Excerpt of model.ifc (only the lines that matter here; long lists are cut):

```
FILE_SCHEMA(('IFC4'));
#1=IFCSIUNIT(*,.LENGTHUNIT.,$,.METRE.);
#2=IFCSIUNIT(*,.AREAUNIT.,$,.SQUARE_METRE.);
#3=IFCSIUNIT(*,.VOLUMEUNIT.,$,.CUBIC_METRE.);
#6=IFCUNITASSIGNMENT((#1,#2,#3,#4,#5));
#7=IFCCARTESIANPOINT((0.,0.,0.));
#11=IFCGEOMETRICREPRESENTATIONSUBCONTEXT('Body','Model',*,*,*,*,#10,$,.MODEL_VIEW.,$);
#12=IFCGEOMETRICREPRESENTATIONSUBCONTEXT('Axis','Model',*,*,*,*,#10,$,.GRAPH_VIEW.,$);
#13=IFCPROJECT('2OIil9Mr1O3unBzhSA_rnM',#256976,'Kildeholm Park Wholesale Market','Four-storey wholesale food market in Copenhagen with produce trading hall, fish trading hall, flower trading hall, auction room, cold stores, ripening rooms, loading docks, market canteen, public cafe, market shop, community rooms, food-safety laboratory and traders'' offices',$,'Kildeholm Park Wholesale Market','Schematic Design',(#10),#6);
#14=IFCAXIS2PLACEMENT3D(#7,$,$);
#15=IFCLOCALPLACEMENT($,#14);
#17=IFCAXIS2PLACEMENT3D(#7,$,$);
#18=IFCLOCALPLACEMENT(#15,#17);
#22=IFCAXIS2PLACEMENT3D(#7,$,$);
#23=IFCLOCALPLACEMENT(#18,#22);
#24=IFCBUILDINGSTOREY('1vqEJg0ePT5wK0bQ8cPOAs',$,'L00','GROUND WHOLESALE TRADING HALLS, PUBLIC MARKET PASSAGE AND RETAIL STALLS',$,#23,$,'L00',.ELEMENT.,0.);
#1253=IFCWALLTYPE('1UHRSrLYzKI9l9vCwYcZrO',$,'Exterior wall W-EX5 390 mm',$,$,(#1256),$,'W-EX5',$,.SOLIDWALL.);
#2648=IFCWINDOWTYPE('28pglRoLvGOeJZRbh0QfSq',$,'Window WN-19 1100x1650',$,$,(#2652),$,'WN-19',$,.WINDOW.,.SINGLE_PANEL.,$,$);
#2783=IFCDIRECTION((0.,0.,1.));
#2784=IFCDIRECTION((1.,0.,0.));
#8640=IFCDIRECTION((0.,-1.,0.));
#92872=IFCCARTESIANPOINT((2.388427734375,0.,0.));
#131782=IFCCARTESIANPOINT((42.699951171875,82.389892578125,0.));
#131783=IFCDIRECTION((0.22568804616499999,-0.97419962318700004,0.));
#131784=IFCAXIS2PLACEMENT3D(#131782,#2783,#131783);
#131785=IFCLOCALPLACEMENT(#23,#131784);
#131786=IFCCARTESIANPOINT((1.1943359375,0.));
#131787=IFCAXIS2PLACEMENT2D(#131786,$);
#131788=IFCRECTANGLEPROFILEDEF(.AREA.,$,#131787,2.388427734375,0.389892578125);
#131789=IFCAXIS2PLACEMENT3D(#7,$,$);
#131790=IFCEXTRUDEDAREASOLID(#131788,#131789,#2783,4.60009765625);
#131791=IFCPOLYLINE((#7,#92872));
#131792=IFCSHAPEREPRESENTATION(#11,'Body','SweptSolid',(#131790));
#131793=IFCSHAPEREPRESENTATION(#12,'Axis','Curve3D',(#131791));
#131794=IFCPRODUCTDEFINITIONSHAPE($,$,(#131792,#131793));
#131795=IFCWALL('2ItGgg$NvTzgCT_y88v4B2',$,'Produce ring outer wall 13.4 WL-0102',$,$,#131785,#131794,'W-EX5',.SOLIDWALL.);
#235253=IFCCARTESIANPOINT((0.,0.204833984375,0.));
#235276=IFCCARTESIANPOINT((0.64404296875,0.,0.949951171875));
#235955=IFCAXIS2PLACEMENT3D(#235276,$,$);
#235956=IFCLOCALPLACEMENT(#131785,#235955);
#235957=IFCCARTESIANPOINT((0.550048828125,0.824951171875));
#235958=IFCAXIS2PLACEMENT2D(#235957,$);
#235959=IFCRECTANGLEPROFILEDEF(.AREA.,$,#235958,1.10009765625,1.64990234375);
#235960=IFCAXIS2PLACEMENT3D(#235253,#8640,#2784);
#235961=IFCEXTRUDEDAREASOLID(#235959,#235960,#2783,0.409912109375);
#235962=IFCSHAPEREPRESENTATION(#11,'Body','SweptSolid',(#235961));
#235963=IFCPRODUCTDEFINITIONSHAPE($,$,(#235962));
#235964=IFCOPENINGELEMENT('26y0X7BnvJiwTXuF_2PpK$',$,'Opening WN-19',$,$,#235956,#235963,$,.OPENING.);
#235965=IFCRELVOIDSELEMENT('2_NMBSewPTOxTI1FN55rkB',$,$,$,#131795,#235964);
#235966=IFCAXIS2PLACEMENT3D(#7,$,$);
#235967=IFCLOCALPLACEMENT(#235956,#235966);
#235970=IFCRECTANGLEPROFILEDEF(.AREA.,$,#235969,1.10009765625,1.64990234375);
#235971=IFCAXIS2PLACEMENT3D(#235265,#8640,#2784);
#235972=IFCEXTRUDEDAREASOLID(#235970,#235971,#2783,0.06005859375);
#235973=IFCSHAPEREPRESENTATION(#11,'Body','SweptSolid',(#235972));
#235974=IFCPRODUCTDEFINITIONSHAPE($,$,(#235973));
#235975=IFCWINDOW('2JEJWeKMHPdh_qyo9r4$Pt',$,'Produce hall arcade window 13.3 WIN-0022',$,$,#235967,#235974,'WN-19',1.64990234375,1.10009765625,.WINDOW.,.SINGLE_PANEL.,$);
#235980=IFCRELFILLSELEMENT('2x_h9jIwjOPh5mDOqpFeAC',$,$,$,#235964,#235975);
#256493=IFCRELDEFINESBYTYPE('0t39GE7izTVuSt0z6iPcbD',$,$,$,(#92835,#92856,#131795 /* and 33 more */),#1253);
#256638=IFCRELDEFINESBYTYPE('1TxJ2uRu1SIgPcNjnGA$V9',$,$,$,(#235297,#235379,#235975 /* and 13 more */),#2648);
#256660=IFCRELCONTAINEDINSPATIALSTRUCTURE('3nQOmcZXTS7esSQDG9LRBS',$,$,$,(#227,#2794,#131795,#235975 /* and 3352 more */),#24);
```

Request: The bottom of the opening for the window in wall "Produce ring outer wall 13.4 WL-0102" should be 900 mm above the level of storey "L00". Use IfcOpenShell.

```python
import numpy as np
import ifcopenshell
import ifcopenshell.api.geometry
import ifcopenshell.geom
import ifcopenshell.util.element
import ifcopenshell.util.placement
import ifcopenshell.util.shape
import ifcopenshell.util.unit

model = ifcopenshell.open("model.ifc")
unit_scale = ifcopenshell.util.unit.calculate_unit_scale(model)

window = model.by_guid("2JEJWeKMHPdh_qyo9r4$Pt")
opening = window.FillsVoids[0].RelatingOpeningElement
storey = ifcopenshell.util.element.get_container(window, ifc_class="IfcBuildingStorey")
level = ifcopenshell.util.placement.get_local_placement(storey.ObjectPlacement)[2, 3]

# The opening's origin need not be at the sill, so measure its lowest point.
shape = ifcopenshell.geom.create_shape(ifcopenshell.geom.settings(), opening)
bottom = ifcopenshell.util.shape.get_shape_bottom_elevation(shape, shape.geometry) / unit_scale
dz = level + 0.9 / unit_scale - bottom

shift = np.array([0.0, 0.0, dz])
# The window is placed relative to its opening, so it follows when the opening moves.
matrix = ifcopenshell.util.placement.get_local_placement(opening.ObjectPlacement)
matrix[:3, 3] += shift
ifcopenshell.api.geometry.edit_object_placement(
    model, product=opening, matrix=matrix, is_si=False, should_transform_children=True
)

print(f"moved by {dz * unit_scale:+.3f} m")

model.write("model_rev.ifc")
```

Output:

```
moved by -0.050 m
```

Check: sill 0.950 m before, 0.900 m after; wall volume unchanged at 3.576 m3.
